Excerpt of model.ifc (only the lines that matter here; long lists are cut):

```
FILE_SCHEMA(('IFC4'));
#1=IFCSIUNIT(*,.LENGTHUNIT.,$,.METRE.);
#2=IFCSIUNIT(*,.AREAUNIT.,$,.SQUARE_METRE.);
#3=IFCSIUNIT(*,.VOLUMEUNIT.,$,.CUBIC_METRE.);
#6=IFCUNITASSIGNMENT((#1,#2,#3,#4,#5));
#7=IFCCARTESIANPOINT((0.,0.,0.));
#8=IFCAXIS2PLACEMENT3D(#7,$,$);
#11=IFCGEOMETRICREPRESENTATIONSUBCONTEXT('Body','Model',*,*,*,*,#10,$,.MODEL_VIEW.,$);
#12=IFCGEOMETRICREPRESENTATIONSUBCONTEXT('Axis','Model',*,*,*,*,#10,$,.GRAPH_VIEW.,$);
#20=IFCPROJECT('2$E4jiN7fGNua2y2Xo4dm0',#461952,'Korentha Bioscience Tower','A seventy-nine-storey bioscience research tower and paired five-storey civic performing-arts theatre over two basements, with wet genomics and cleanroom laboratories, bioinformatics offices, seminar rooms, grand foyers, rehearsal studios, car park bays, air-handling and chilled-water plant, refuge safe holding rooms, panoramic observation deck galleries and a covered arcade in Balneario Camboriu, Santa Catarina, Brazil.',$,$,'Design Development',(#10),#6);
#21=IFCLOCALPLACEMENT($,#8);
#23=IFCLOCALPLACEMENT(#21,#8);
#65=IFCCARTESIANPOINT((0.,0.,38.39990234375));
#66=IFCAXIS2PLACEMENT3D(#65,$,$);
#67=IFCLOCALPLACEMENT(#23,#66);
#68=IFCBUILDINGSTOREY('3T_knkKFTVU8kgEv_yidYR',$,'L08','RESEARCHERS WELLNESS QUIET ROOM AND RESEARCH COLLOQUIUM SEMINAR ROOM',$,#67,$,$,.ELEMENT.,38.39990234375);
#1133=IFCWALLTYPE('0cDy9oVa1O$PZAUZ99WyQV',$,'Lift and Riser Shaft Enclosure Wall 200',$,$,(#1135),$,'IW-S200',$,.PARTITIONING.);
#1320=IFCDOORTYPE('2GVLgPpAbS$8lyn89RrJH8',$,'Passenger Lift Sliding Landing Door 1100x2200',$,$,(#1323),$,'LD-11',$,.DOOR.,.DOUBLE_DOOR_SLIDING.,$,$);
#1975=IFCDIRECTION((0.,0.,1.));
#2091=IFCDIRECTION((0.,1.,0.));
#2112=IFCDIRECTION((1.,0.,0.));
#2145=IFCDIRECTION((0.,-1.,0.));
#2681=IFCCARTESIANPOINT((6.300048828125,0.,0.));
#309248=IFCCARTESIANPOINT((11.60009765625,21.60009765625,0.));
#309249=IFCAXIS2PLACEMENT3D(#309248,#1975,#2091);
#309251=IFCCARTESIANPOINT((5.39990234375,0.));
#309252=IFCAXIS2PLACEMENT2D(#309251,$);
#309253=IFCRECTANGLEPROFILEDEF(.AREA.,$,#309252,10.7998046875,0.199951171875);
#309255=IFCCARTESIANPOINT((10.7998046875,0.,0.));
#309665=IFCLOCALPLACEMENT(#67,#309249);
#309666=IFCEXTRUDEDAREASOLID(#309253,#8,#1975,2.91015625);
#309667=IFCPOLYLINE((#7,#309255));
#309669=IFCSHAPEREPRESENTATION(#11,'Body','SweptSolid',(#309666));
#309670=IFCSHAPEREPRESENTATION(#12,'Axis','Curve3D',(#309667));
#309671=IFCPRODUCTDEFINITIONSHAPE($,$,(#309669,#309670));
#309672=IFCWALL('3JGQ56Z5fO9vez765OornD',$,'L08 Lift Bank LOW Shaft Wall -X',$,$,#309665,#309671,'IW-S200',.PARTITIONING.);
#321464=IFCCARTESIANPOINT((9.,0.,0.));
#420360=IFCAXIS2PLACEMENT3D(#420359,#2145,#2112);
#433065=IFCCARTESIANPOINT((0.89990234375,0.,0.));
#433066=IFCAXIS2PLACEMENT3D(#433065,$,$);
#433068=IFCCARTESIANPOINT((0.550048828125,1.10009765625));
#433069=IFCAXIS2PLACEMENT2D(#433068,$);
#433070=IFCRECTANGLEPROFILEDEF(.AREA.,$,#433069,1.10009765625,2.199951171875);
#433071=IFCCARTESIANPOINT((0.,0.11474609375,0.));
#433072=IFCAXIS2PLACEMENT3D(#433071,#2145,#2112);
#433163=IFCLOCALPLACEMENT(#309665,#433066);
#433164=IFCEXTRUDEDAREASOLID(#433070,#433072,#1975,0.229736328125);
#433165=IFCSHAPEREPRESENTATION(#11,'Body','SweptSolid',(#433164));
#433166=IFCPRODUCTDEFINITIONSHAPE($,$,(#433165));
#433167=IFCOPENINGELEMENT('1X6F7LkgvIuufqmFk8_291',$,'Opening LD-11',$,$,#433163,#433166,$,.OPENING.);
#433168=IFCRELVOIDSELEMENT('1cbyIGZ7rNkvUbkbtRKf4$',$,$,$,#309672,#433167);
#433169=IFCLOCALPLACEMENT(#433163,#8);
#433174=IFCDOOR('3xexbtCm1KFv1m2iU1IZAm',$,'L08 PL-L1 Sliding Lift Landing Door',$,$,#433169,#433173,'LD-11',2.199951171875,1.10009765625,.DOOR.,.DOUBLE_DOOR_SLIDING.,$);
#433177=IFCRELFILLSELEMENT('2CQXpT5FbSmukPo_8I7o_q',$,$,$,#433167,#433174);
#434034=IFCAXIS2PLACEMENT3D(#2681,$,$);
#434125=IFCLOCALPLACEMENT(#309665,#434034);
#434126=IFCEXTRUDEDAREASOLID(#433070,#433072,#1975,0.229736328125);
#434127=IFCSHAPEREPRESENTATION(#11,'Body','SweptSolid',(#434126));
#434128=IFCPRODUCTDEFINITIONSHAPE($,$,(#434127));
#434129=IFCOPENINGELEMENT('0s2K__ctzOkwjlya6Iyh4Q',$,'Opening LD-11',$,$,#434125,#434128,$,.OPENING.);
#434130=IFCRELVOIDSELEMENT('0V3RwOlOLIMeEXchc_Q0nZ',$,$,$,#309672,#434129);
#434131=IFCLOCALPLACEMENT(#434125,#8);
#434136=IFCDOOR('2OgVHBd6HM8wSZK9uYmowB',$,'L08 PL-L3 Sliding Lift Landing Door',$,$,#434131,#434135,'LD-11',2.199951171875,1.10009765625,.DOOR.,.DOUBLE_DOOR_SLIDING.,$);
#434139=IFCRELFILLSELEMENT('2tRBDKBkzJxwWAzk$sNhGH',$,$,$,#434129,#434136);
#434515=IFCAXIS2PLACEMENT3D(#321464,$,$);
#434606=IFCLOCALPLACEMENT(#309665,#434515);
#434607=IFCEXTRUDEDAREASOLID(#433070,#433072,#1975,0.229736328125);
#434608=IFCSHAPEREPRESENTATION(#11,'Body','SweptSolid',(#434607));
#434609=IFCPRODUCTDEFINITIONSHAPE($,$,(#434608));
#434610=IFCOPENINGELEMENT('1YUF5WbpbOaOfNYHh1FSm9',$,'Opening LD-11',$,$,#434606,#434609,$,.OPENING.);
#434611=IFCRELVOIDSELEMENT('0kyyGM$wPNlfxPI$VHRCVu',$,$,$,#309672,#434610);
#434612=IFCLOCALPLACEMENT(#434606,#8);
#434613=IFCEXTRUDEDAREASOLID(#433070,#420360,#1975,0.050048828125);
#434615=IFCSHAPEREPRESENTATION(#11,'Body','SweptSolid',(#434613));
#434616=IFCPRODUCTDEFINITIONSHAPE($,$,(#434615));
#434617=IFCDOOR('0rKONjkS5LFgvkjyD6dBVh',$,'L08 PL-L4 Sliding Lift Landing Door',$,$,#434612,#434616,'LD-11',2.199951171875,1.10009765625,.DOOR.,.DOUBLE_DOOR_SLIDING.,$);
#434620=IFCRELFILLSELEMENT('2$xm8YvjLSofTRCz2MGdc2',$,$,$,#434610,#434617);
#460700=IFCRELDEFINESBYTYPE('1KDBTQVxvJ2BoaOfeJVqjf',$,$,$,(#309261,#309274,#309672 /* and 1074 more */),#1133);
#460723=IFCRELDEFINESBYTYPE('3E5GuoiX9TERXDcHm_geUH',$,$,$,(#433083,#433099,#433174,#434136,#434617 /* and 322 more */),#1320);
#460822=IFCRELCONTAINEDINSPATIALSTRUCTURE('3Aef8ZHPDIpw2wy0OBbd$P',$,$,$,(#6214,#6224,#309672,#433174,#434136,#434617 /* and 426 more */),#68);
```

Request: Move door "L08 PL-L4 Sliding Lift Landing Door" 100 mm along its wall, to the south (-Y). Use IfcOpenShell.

```python
import ifcopenshell
import ifcopenshell.api.geometry
import ifcopenshell.util.placement

model = ifcopenshell.open("model.ifc")

door = model.by_guid("0rKONjkS5LFgvkjyD6dBVh")
opening = door.FillsVoids[0].RelatingOpeningElement
wall = opening.VoidsElements[0].RelatingBuildingElement

wall_matrix = ifcopenshell.util.placement.get_local_placement(wall.ObjectPlacement)
shift = wall_matrix[:3, 0] * -0.1
before = ifcopenshell.util.placement.get_local_placement(door.ObjectPlacement)[:3, 3].copy()

# The door is placed relative to its opening, so it follows when the opening moves.
matrix = ifcopenshell.util.placement.get_local_placement(opening.ObjectPlacement)
matrix[:3, 3] += shift
ifcopenshell.api.geometry.edit_object_placement(
    model, product=opening, matrix=matrix, is_si=False, should_transform_children=True
)

after = ifcopenshell.util.placement.get_local_placement(door.ObjectPlacement)[:3, 3]
print("door moved by", (after - before).round(3) + 0.0)

model.write("model_v2.ifc")
```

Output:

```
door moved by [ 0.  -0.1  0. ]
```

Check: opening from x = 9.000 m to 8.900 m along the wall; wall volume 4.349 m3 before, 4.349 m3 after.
